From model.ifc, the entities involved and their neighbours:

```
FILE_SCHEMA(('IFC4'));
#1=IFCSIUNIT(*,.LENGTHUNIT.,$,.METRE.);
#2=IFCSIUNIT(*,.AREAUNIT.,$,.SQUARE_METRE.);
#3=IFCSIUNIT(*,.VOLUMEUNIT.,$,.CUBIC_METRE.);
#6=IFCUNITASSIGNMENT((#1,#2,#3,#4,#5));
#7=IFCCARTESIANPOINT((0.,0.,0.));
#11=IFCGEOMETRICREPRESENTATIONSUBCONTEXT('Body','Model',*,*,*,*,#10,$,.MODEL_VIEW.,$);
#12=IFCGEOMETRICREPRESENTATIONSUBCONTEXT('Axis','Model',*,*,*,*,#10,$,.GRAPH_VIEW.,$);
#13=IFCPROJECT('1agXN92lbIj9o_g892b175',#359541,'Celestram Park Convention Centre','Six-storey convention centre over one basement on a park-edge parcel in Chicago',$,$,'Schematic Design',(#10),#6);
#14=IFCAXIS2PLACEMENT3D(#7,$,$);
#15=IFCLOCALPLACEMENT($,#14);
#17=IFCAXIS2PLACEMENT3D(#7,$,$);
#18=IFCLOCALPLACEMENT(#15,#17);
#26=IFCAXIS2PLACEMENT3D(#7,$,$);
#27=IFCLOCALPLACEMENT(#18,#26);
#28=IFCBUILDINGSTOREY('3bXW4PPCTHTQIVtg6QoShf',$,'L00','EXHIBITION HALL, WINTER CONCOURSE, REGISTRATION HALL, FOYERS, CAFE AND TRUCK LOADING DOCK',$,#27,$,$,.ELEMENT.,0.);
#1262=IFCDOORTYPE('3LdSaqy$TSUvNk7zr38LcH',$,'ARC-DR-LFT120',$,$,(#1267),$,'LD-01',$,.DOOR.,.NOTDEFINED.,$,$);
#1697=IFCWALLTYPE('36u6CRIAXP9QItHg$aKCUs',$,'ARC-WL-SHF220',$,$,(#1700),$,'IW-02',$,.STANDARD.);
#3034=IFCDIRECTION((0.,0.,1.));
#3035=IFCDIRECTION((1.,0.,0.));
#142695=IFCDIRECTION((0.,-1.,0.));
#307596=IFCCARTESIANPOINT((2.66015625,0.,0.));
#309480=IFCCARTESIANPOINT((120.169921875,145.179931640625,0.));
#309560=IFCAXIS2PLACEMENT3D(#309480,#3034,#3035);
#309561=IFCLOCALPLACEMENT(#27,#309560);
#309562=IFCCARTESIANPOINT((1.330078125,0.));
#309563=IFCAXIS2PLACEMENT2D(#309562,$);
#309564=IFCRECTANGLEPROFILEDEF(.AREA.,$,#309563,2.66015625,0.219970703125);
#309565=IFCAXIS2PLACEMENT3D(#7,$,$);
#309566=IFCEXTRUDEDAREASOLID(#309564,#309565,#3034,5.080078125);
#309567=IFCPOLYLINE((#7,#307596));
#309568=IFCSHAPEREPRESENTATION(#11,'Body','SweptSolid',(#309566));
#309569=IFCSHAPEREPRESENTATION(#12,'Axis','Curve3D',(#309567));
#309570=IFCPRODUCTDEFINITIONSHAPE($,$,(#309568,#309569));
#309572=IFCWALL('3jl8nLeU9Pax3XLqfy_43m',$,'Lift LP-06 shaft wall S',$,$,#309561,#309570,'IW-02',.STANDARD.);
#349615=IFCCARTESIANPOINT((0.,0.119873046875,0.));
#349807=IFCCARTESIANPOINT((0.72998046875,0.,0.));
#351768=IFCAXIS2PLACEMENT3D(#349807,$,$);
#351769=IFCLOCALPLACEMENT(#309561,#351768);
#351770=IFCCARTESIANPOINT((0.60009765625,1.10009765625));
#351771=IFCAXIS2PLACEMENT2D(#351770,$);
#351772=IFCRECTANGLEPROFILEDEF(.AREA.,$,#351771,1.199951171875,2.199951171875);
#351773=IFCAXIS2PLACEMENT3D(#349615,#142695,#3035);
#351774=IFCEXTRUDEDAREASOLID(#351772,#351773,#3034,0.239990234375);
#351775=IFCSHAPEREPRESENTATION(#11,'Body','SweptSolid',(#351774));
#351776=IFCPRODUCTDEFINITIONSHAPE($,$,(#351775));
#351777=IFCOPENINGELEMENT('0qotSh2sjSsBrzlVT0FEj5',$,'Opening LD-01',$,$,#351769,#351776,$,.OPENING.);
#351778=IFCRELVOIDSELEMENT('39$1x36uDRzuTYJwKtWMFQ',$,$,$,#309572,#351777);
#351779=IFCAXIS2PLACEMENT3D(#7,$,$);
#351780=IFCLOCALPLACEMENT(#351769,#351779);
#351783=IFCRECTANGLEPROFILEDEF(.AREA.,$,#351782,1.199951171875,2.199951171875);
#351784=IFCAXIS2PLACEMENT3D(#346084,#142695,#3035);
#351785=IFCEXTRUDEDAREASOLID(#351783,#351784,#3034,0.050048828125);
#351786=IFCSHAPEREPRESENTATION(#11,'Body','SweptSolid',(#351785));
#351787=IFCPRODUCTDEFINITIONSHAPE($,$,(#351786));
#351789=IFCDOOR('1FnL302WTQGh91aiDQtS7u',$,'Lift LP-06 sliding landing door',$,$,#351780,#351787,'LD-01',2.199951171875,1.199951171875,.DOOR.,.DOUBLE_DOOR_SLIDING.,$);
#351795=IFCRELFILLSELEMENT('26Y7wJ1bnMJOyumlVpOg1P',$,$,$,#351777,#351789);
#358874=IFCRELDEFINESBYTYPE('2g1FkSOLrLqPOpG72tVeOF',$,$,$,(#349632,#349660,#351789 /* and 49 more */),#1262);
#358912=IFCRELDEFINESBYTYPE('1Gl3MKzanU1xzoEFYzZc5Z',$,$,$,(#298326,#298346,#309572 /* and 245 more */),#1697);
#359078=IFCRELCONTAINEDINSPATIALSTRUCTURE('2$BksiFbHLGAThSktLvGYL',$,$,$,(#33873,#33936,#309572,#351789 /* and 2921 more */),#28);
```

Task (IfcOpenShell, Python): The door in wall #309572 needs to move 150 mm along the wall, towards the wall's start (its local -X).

```python
import ifcopenshell
import ifcopenshell.api.geometry
import ifcopenshell.util.placement
import ifcopenshell.util.unit

model = ifcopenshell.open("model.ifc")
unit_scale = ifcopenshell.util.unit.calculate_unit_scale(model)

door = model.by_guid("1FnL302WTQGh91aiDQtS7u")
opening = door.FillsVoids[0].RelatingOpeningElement
wall = opening.VoidsElements[0].RelatingBuildingElement

wall_matrix = ifcopenshell.util.placement.get_local_placement(wall.ObjectPlacement)
shift = wall_matrix[:3, 0] * -0.15 / unit_scale
before = ifcopenshell.util.placement.get_local_placement(door.ObjectPlacement)[:3, 3].copy()

# The door is placed relative to its opening, so it follows when the opening moves.
matrix = ifcopenshell.util.placement.get_local_placement(opening.ObjectPlacement)
matrix[:3, 3] += shift
ifcopenshell.api.geometry.edit_object_placement(
    model, product=opening, matrix=matrix, is_si=False, should_transform_children=True
)

after = ifcopenshell.util.placement.get_local_placement(door.ObjectPlacement)[:3, 3]
print("door moved by", (after - before).round(3) + 0.0)

model.write("model_updated.ifc")
```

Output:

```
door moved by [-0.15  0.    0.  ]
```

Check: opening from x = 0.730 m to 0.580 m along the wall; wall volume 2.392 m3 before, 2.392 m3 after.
